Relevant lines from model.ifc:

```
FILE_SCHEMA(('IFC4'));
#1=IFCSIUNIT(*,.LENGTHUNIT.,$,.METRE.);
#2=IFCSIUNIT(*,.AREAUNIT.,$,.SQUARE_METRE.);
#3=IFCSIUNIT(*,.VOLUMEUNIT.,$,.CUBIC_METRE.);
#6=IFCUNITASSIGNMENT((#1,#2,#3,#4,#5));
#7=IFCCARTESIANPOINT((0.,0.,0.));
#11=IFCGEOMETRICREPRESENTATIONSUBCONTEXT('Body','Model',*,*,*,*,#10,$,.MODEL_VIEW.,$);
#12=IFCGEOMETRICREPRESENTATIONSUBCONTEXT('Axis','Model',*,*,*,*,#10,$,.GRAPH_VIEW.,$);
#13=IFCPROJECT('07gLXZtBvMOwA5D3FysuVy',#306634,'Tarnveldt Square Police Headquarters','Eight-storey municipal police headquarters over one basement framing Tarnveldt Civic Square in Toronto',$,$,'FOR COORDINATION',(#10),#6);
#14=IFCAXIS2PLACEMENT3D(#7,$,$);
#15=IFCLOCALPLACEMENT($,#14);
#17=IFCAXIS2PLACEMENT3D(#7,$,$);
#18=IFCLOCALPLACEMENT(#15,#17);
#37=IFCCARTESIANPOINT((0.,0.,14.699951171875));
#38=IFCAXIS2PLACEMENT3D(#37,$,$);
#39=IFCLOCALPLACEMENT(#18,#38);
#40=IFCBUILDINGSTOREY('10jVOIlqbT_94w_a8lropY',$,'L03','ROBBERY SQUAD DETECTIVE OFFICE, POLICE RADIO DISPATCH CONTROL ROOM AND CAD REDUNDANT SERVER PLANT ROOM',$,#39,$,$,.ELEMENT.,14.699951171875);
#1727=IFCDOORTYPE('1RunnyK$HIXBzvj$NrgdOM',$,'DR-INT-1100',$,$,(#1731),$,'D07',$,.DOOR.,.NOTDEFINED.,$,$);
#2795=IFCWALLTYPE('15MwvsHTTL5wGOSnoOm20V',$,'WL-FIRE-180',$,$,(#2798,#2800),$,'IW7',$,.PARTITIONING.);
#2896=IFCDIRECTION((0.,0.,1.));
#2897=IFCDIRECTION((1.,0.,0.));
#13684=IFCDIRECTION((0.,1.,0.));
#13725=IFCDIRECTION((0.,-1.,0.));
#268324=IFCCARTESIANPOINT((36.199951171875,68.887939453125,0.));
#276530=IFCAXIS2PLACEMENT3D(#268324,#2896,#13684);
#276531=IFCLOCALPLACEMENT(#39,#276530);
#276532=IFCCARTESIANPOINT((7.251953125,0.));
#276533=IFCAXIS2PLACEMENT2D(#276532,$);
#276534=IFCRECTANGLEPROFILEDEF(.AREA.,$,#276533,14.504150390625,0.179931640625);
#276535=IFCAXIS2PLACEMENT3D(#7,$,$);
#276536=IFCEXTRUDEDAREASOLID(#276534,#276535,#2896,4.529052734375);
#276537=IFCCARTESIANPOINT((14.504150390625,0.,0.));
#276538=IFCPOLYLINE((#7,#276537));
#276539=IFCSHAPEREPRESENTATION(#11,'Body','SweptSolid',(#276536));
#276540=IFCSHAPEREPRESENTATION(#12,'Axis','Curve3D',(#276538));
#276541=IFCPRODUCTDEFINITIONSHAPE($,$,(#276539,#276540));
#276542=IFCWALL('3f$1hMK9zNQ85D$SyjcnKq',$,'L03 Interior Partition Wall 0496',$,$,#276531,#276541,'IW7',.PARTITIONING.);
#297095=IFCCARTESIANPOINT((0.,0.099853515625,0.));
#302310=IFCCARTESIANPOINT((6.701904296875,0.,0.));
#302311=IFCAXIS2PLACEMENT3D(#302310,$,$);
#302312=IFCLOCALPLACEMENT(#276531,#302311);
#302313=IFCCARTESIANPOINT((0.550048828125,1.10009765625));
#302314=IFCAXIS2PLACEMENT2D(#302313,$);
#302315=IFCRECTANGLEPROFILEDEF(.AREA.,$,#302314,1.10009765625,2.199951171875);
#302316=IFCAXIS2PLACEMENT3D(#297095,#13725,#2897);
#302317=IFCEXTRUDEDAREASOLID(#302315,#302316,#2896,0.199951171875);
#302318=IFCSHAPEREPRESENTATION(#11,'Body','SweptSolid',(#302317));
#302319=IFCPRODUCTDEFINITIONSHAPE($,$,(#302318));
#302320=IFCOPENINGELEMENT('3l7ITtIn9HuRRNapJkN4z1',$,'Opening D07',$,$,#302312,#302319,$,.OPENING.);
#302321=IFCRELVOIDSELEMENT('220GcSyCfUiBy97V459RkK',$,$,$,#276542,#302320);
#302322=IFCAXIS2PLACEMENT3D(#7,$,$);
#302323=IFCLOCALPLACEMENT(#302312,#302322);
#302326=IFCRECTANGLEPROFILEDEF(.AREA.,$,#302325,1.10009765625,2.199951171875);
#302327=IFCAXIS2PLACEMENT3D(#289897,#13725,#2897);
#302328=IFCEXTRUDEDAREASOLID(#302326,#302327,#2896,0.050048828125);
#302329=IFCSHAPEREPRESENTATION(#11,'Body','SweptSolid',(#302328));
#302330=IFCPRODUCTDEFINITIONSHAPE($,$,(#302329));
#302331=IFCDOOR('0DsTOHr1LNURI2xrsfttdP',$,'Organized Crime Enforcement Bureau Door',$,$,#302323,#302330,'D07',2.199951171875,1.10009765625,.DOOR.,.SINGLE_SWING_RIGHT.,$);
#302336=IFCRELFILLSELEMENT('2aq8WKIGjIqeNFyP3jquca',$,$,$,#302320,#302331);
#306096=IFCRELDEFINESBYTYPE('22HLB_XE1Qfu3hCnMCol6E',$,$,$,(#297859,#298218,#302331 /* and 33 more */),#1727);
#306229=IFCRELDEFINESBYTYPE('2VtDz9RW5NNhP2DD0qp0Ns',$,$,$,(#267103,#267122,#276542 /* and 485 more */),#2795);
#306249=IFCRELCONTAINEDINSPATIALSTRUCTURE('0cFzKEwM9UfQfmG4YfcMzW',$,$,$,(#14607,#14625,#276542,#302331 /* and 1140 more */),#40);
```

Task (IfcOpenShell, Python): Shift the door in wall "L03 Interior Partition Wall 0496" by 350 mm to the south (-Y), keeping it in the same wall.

```python
import ifcopenshell
import ifcopenshell.api.geometry
import ifcopenshell.util.placement
import ifcopenshell.util.unit

model = ifcopenshell.open("model.ifc")
unit_scale = ifcopenshell.util.unit.calculate_unit_scale(model)

door = model.by_id(302331)
opening = door.FillsVoids[0].RelatingOpeningElement
wall = opening.VoidsElements[0].RelatingBuildingElement

wall_matrix = ifcopenshell.util.placement.get_local_placement(wall.ObjectPlacement)
shift = wall_matrix[:3, 0] * -0.35 / unit_scale
before = ifcopenshell.util.placement.get_local_placement(door.ObjectPlacement)[:3, 3].copy()

# The door is placed relative to its opening, so it follows when the opening moves.
matrix = ifcopenshell.util.placement.get_local_placement(opening.ObjectPlacement)
matrix[:3, 3] += shift
ifcopenshell.api.geometry.edit_object_placement(
    model, product=opening, matrix=matrix, is_si=False, should_transform_children=True
)

after = ifcopenshell.util.placement.get_local_placement(door.ObjectPlacement)[:3, 3]
print("door moved by", (after - before).round(3) + 0.0)

model.write("model_v2.ifc")
```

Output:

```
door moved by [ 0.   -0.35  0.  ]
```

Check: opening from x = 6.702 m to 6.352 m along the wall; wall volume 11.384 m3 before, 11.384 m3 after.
